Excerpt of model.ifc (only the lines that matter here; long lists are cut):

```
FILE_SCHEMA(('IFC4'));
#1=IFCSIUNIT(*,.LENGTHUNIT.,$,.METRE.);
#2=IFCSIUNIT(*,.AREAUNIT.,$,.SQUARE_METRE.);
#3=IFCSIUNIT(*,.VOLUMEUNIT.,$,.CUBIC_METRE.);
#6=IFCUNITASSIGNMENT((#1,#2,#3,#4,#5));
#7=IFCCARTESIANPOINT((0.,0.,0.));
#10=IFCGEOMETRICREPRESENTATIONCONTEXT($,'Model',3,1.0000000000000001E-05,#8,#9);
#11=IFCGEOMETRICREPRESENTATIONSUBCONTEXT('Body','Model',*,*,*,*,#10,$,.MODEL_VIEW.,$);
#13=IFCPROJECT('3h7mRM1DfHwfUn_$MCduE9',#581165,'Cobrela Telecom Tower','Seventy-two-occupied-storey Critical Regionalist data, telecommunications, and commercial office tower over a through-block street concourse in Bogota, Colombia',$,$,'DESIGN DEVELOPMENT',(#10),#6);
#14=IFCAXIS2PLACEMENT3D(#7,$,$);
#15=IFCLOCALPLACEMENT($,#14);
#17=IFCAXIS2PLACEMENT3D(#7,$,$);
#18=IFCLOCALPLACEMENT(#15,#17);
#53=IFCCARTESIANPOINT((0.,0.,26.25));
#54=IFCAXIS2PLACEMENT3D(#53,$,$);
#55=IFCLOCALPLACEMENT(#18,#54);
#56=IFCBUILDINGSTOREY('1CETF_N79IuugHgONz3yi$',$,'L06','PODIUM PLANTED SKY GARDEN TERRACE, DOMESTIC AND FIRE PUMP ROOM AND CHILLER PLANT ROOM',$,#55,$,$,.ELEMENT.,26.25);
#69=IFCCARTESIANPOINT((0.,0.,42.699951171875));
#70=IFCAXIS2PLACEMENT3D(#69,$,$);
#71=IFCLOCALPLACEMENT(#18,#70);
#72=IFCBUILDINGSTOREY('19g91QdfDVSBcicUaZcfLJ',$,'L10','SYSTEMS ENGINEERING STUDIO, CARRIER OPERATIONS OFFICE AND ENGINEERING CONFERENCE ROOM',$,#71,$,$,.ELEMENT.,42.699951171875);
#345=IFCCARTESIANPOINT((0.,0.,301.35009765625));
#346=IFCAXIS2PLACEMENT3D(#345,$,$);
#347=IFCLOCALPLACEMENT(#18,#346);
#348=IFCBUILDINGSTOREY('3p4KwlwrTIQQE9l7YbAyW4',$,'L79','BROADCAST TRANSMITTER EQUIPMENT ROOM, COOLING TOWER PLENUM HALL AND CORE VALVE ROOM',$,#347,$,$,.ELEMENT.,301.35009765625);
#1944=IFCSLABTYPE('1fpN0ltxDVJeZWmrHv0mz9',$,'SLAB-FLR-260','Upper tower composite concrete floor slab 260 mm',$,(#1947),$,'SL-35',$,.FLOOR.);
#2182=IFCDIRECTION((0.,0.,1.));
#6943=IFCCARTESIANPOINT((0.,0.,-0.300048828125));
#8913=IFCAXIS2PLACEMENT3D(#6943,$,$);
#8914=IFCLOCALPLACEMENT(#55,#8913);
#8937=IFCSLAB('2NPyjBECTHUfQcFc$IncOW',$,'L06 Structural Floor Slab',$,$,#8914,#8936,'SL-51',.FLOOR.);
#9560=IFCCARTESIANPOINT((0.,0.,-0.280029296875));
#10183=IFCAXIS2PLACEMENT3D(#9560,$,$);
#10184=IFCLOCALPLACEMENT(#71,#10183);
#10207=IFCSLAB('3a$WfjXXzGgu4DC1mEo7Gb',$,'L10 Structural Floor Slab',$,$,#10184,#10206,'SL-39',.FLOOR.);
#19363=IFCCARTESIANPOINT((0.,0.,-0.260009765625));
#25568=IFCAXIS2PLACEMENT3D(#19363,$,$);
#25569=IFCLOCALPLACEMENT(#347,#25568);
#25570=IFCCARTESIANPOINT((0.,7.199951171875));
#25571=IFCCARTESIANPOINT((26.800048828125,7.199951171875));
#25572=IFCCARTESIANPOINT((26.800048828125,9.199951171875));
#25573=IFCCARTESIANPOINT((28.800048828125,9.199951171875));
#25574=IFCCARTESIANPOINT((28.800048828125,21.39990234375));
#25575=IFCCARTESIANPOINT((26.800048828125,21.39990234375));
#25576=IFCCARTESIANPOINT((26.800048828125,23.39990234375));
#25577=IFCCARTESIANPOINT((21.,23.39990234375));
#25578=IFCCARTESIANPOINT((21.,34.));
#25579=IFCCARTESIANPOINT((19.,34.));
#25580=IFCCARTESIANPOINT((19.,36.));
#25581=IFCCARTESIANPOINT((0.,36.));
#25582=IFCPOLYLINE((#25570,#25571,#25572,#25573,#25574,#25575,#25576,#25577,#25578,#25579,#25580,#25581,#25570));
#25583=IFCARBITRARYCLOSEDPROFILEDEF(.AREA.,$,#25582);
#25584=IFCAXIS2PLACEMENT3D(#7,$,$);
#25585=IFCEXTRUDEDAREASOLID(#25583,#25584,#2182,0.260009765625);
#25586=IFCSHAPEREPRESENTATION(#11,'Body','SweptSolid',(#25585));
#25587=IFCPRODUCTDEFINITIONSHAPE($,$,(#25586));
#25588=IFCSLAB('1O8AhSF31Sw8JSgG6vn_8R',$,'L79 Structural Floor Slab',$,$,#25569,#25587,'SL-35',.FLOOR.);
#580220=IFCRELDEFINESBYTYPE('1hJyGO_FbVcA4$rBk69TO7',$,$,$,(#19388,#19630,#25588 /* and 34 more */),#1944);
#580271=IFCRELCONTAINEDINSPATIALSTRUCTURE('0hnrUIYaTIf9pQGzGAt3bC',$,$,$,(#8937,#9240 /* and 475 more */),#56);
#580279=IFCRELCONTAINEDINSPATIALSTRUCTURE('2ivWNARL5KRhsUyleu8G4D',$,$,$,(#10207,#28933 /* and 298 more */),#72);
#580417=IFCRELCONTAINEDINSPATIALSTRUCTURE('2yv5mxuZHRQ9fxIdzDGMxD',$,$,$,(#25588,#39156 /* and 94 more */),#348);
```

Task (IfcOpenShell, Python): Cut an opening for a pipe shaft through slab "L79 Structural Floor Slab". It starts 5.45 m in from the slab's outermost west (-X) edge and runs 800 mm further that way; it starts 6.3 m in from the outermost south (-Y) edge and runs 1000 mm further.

```python
import numpy as np
import ifcopenshell
import ifcopenshell.api.feature
import ifcopenshell.api.geometry
import ifcopenshell.api.root
import ifcopenshell.geom
import ifcopenshell.util.placement
import ifcopenshell.util.representation
import ifcopenshell.util.shape
import ifcopenshell.util.unit

model = ifcopenshell.open("model.ifc")
unit_scale = ifcopenshell.util.unit.calculate_unit_scale(model)
settings = ifcopenshell.geom.settings()


def volume(element):
    """Net volume in cubic metres, openings subtracted."""
    shape = ifcopenshell.geom.create_shape(settings, element)
    return ifcopenshell.util.shape.get_volume(shape.geometry)


slab = model.by_guid("1O8AhSF31Sw8JSgG6vn_8R")
before = volume(slab)

# Extent in the slab's own axes, in metres. The edges named are its -X and -Y sides.
slab_shape = ifcopenshell.geom.create_shape(settings, slab)
vertices = ifcopenshell.util.shape.get_vertices(slab_shape.geometry)
x_min, y_min, bottom = vertices.min(axis=0)
top = vertices[:, 2].max()

opening = ifcopenshell.api.root.create_entity(model, ifc_class="IfcOpeningElement", name="Pipe shaft opening", predefined_type="OPENING")
context = ifcopenshell.util.representation.get_context(model, "Model", "Body", "MODEL_VIEW")
width, depth = 0.8, 1
outline = [(0.0, 0.0), (width, 0.0), (width, depth), (0.0, depth), (0.0, 0.0)]
# Overshoot both faces by 50 mm so the cut is clean.
shape = ifcopenshell.api.geometry.add_slab_representation(
    model, context=context, depth=top - bottom + 0.1, polyline=outline
)
ifcopenshell.api.geometry.assign_representation(model, product=opening, representation=shape)

matrix = ifcopenshell.util.placement.get_local_placement(slab.ObjectPlacement)
matrix[:, 3] = matrix @ np.append(np.array([x_min + 5.45, y_min + 6.3, bottom - 0.05]) / unit_scale, 1.0)
ifcopenshell.api.geometry.edit_object_placement(model, product=opening, matrix=matrix, is_si=False)
ifcopenshell.api.feature.add_feature(model, feature=opening, element=slab)

after = volume(slab)

print(f"slab volume {before:.3f} -> {after:.3f} m3")

model.write("model_updated.ifc")
```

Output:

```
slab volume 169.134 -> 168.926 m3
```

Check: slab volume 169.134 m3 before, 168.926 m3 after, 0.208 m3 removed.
